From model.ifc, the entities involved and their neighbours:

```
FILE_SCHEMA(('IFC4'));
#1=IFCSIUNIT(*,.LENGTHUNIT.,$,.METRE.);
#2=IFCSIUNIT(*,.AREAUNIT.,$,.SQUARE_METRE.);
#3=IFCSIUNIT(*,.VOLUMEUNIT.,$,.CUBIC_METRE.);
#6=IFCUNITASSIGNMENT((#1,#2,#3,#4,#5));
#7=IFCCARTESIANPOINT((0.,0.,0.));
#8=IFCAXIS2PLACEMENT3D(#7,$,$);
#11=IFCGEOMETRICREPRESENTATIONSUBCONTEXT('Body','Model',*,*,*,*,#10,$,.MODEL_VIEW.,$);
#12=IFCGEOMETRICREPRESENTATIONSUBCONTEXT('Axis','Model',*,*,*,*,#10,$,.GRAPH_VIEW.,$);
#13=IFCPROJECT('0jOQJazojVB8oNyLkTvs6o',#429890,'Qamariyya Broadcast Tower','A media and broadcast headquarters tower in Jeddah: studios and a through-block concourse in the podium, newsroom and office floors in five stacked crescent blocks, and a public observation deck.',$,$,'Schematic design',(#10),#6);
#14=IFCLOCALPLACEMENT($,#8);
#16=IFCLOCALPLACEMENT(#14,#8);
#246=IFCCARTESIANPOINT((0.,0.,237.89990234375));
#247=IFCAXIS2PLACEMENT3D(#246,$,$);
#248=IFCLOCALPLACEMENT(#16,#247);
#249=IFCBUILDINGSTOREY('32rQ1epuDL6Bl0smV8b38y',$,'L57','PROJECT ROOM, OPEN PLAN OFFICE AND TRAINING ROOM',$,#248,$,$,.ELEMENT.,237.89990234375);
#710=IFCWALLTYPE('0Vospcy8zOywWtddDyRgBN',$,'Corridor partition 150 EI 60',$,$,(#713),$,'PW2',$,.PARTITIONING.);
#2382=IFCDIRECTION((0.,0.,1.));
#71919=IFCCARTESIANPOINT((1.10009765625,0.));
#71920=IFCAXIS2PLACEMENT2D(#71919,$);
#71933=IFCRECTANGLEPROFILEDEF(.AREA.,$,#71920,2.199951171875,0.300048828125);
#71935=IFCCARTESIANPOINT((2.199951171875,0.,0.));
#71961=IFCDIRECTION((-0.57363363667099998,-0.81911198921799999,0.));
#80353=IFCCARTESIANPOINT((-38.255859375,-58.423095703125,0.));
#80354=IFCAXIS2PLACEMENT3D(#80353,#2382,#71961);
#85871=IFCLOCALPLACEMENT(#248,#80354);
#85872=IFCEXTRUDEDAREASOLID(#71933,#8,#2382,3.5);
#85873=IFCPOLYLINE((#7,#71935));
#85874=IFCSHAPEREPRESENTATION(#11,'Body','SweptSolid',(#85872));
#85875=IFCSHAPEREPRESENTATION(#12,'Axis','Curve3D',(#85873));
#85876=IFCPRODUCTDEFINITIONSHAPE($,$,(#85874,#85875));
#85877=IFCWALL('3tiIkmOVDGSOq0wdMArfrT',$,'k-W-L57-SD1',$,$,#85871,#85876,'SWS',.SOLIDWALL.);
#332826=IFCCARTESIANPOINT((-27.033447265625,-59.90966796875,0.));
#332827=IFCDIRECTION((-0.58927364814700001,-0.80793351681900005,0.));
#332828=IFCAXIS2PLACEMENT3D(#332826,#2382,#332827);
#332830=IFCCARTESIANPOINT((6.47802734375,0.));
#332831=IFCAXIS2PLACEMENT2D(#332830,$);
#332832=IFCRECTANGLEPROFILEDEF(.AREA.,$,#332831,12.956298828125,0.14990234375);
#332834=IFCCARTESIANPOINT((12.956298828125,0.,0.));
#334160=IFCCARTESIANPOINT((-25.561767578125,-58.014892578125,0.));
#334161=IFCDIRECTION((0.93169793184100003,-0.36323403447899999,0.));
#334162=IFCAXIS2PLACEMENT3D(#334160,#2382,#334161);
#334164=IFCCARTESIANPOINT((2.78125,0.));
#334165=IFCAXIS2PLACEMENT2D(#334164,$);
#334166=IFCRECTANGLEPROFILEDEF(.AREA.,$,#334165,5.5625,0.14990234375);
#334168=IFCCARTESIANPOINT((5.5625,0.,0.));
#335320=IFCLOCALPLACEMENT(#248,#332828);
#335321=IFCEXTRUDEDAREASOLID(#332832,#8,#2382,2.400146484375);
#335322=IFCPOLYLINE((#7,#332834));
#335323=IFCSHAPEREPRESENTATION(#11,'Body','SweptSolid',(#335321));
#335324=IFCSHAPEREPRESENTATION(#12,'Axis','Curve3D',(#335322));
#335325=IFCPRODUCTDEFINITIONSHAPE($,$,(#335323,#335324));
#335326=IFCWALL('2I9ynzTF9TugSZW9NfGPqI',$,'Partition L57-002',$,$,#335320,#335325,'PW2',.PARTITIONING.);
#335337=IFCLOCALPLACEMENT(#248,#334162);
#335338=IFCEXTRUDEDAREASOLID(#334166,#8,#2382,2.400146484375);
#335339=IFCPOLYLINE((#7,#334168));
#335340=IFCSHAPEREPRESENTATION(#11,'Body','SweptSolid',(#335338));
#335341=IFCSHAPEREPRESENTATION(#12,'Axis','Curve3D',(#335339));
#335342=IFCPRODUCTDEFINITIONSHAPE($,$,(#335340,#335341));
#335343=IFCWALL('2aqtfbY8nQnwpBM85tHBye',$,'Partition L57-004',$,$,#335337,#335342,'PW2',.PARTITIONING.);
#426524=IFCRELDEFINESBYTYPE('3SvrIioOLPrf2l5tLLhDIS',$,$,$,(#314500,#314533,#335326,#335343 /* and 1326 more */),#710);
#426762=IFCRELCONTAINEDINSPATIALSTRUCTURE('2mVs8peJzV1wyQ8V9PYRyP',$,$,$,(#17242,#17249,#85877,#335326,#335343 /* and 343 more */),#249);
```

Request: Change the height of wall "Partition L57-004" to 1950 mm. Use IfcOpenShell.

```python
import ifcopenshell
import ifcopenshell.geom
import ifcopenshell.util.representation
import ifcopenshell.util.shape

model = ifcopenshell.open("model.ifc")
settings = ifcopenshell.geom.settings()


def volume(element):
    """Net volume in cubic metres, openings subtracted."""
    shape = ifcopenshell.geom.create_shape(settings, element)
    return ifcopenshell.util.shape.get_volume(shape.geometry)


wall = model.by_guid("2aqtfbY8nQnwpBM85tHBye")
before = volume(wall)

body = ifcopenshell.util.representation.get_representation(wall, "Model", "Body")
solid = body.Items[0]
old_height = solid.Depth
solid.Depth = 1.95
after = volume(wall)

print(f"height {old_height:g} -> {solid.Depth:g}, volume {before:.3f} -> {after:.3f} m3")

model.write("model_updated.ifc")
```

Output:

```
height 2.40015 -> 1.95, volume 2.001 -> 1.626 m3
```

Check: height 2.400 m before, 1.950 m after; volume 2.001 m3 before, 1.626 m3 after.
